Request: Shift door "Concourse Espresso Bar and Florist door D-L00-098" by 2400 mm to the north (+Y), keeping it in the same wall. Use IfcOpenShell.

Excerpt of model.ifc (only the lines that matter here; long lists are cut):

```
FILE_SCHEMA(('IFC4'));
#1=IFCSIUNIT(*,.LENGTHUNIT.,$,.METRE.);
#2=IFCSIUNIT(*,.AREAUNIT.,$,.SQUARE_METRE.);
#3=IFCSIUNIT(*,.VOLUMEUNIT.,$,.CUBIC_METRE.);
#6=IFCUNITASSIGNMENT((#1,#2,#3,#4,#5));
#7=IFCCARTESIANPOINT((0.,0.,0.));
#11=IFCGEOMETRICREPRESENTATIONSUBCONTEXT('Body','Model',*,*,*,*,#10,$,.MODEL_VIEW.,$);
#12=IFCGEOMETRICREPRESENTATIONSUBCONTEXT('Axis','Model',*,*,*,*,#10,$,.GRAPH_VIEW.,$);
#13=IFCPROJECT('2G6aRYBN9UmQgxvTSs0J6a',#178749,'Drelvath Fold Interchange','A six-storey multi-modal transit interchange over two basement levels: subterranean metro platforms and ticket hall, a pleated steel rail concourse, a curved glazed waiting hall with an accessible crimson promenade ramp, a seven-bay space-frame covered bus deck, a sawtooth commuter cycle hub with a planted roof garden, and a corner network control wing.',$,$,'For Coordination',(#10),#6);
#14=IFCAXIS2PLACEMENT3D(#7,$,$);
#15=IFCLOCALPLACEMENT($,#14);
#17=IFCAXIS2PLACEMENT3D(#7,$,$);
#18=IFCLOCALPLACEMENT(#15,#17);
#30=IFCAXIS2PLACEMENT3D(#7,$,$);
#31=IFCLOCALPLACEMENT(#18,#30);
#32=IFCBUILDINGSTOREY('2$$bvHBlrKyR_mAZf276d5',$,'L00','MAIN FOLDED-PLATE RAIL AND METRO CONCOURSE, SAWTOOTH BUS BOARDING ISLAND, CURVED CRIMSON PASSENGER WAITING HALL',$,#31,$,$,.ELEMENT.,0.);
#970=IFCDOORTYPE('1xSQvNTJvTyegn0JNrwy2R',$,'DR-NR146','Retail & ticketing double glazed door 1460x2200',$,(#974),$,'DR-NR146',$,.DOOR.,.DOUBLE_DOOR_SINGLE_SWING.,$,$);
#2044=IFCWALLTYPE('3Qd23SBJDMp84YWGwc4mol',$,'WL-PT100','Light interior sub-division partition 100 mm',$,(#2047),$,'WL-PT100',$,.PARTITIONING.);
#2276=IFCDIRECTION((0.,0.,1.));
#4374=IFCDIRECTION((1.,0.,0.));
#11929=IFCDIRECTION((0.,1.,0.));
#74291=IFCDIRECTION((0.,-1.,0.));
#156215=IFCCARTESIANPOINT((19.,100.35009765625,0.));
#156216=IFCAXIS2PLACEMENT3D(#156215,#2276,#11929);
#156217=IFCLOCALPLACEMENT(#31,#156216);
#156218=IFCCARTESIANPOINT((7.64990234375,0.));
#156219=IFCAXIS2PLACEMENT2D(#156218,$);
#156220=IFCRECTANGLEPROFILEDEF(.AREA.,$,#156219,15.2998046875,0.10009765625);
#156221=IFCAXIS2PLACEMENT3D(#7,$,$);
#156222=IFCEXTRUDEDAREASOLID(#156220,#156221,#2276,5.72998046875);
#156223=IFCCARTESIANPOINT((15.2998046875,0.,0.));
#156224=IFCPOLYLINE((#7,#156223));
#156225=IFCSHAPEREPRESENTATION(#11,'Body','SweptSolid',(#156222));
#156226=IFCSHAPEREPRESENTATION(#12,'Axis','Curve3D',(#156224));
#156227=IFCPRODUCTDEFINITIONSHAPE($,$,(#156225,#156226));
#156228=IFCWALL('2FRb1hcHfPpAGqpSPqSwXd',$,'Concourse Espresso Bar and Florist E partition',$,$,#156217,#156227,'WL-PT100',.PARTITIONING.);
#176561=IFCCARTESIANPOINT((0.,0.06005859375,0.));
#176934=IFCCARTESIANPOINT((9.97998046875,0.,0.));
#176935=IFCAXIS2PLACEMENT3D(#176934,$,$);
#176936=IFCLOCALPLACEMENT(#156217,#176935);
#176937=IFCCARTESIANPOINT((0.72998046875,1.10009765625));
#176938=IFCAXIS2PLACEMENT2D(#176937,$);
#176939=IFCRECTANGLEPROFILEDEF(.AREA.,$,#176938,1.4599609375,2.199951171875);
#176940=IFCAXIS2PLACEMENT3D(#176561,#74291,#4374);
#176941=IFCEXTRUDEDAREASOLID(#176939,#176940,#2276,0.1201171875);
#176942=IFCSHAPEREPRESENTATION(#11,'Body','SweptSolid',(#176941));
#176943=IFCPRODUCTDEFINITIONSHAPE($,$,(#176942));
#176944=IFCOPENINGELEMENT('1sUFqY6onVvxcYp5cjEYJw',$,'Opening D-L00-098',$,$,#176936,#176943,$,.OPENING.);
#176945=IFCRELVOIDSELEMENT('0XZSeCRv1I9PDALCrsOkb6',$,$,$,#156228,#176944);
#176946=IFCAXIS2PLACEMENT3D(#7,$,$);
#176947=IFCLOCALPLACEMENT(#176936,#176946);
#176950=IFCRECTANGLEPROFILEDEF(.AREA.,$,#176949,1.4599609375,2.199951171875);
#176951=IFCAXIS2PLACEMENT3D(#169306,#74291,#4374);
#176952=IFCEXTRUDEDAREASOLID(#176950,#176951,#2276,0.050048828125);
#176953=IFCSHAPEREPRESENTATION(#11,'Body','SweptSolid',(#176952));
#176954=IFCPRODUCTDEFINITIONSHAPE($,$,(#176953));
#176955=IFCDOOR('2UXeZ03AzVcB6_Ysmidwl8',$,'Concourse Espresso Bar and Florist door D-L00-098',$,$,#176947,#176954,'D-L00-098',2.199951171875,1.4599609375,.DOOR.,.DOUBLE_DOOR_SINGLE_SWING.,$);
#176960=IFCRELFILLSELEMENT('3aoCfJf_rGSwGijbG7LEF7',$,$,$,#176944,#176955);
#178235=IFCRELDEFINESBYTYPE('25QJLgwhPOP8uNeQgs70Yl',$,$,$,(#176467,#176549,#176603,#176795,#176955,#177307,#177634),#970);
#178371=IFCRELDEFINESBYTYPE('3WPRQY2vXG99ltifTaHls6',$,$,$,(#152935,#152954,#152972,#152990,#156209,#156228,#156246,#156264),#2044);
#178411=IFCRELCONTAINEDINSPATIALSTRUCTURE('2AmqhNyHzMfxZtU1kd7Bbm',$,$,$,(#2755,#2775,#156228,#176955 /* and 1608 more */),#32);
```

```python
import ifcopenshell
import ifcopenshell.api.geometry
import ifcopenshell.util.placement

model = ifcopenshell.open("model.ifc")

door = model.by_id(176955)
opening = door.FillsVoids[0].RelatingOpeningElement
wall = opening.VoidsElements[0].RelatingBuildingElement

wall_matrix = ifcopenshell.util.placement.get_local_placement(wall.ObjectPlacement)
shift = wall_matrix[:3, 0] * 2.4
before = ifcopenshell.util.placement.get_local_placement(door.ObjectPlacement)[:3, 3].copy()

# The door is placed relative to its opening, so it follows when the opening moves.
matrix = ifcopenshell.util.placement.get_local_placement(opening.ObjectPlacement)
matrix[:3, 3] += shift
ifcopenshell.api.geometry.edit_object_placement(
    model, product=opening, matrix=matrix, is_si=False, should_transform_children=True
)

after = ifcopenshell.util.placement.get_local_placement(door.ObjectPlacement)[:3, 3]
print("door moved by", (after - before).round(3) + 0.0)

model.write("model_v2.ifc")
```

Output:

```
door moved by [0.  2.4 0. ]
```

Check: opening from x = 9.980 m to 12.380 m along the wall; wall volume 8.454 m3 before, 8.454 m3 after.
